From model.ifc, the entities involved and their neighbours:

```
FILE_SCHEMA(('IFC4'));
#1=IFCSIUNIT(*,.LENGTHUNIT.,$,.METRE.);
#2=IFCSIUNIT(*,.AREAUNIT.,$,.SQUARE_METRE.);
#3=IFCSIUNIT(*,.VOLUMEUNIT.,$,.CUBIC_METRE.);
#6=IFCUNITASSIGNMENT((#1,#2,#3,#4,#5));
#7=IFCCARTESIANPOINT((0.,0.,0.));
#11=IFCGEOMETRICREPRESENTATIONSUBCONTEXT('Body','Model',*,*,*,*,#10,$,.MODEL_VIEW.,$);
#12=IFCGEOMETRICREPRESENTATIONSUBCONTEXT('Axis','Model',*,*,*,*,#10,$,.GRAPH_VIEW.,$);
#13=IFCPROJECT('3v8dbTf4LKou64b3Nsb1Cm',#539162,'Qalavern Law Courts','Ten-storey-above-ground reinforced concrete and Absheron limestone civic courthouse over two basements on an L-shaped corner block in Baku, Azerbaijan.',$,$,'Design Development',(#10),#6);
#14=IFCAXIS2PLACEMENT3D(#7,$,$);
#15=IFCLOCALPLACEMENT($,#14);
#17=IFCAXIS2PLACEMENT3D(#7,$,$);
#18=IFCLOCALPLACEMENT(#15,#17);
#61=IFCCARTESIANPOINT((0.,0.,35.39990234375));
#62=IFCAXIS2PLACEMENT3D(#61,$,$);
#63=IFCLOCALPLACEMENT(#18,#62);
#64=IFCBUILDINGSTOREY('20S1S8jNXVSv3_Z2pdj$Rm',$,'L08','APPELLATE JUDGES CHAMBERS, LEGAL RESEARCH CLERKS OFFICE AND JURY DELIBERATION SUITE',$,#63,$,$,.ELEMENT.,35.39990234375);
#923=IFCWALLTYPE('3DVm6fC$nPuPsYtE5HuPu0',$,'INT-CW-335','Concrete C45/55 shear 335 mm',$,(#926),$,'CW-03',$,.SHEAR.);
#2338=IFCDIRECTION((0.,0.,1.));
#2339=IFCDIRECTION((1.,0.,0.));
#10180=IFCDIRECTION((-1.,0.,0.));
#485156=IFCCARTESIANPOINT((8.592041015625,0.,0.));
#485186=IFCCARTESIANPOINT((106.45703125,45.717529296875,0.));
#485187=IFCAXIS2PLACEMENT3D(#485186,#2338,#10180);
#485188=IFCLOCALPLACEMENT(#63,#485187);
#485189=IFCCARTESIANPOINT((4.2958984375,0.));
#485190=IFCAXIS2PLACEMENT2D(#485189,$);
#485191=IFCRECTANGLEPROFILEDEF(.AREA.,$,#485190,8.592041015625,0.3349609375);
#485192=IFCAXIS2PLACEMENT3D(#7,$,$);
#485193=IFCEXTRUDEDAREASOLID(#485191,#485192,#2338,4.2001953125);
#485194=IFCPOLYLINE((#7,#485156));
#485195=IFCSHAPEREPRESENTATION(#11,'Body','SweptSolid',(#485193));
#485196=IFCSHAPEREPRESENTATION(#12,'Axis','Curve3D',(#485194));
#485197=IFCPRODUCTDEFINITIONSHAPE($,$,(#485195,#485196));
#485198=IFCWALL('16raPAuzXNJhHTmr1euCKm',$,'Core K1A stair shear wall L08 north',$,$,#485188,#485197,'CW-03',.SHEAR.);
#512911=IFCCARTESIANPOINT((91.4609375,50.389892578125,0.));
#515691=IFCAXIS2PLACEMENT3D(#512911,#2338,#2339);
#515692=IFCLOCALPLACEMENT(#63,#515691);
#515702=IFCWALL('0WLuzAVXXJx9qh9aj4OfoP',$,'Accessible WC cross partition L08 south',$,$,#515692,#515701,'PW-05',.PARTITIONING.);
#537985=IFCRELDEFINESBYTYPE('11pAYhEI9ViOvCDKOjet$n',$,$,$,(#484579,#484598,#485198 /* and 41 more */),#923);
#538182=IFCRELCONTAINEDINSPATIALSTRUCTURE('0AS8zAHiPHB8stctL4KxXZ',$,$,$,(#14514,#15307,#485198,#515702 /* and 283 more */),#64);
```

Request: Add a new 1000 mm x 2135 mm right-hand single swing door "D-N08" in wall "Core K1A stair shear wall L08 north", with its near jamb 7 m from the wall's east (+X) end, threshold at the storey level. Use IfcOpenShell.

```python
import numpy as np
import ifcopenshell
import ifcopenshell.api.feature
import ifcopenshell.api.geometry
import ifcopenshell.api.root
import ifcopenshell.api.spatial
import ifcopenshell.geom
import ifcopenshell.util.element
import ifcopenshell.util.placement
import ifcopenshell.util.representation
import ifcopenshell.util.shape
import ifcopenshell.util.unit

model = ifcopenshell.open("model.ifc")
unit_scale = ifcopenshell.util.unit.calculate_unit_scale(model)
settings = ifcopenshell.geom.settings()


def volume(element):
    """Net volume in cubic metres, openings subtracted."""
    shape = ifcopenshell.geom.create_shape(settings, element)
    return ifcopenshell.util.shape.get_volume(shape.geometry)


wall = model.by_guid("16raPAuzXNJhHTmr1euCKm")
storey = ifcopenshell.util.element.get_container(wall, ifc_class="IfcBuildingStorey")
context = ifcopenshell.util.representation.get_context(model, "Model", "Body", "MODEL_VIEW")
before = volume(wall)

width, height, from_end, sill = 1, 2.135, 7, 0.0  # metres

# The wall runs along its own X axis, and the end named is its -X end.
wall_shape = ifcopenshell.geom.create_shape(settings, wall)
x, y, z = ifcopenshell.util.shape.get_vertices(wall_shape.geometry).T
start = x.min() + from_end
face, thickness = float(y.min()), float(y.max() - y.min())
wall_matrix = ifcopenshell.util.placement.get_local_placement(wall.ObjectPlacement)
level = ifcopenshell.util.placement.get_local_placement(storey.ObjectPlacement)[2, 3]


def in_wall(x, y):
    """Placement at x, y metres in the wall's axes, at sill height."""
    matrix = wall_matrix.copy()
    matrix[:, 3] = wall_matrix @ np.array([x / unit_scale, y / unit_scale, 0.0, 1.0])
    matrix[2, 3] = level + sill / unit_scale
    return matrix


# Opening: a box that overshoots both wall faces by 50 mm.
opening = ifcopenshell.api.root.create_entity(model, ifc_class="IfcOpeningElement", predefined_type="OPENING")
box = ifcopenshell.api.geometry.add_wall_representation(
    model, context=context, length=width, height=height, thickness=thickness + 0.1
)
ifcopenshell.api.geometry.assign_representation(model, product=opening, representation=box)
ifcopenshell.api.geometry.edit_object_placement(model, product=opening, matrix=in_wall(start, face - 0.05), is_si=False)
ifcopenshell.api.feature.add_feature(model, feature=opening, element=wall)

door = ifcopenshell.api.root.create_entity(model, ifc_class="IfcDoor", name="D-N08", predefined_type="DOOR")
door.OverallWidth, door.OverallHeight = width / unit_scale, height / unit_scale
door.OperationType = "SINGLE_SWING_RIGHT"
body = ifcopenshell.api.geometry.add_door_representation(
    model,
    context=context,
    overall_width=door.OverallWidth,
    overall_height=door.OverallHeight,
    operation_type="SINGLE_SWING_RIGHT",
    lining_properties={"LiningDepth": thickness / unit_scale, "ThresholdDepth": thickness / unit_scale},
)
ifcopenshell.api.geometry.assign_representation(model, product=door, representation=body)
ifcopenshell.api.spatial.assign_container(model, products=[door], relating_structure=storey)
ifcopenshell.api.feature.add_filling(model, opening=opening, element=door)

# The lining spans the wall, so the door starts at the wall face.
ifcopenshell.api.geometry.edit_object_placement(model, product=door, matrix=in_wall(start, face), is_si=False)

after = volume(wall)

print(f"wall volume {before:.3f} -> {after:.3f} m3")

model.write("model_updated.ifc")
```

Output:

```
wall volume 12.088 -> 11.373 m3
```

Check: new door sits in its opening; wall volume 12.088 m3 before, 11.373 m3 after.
